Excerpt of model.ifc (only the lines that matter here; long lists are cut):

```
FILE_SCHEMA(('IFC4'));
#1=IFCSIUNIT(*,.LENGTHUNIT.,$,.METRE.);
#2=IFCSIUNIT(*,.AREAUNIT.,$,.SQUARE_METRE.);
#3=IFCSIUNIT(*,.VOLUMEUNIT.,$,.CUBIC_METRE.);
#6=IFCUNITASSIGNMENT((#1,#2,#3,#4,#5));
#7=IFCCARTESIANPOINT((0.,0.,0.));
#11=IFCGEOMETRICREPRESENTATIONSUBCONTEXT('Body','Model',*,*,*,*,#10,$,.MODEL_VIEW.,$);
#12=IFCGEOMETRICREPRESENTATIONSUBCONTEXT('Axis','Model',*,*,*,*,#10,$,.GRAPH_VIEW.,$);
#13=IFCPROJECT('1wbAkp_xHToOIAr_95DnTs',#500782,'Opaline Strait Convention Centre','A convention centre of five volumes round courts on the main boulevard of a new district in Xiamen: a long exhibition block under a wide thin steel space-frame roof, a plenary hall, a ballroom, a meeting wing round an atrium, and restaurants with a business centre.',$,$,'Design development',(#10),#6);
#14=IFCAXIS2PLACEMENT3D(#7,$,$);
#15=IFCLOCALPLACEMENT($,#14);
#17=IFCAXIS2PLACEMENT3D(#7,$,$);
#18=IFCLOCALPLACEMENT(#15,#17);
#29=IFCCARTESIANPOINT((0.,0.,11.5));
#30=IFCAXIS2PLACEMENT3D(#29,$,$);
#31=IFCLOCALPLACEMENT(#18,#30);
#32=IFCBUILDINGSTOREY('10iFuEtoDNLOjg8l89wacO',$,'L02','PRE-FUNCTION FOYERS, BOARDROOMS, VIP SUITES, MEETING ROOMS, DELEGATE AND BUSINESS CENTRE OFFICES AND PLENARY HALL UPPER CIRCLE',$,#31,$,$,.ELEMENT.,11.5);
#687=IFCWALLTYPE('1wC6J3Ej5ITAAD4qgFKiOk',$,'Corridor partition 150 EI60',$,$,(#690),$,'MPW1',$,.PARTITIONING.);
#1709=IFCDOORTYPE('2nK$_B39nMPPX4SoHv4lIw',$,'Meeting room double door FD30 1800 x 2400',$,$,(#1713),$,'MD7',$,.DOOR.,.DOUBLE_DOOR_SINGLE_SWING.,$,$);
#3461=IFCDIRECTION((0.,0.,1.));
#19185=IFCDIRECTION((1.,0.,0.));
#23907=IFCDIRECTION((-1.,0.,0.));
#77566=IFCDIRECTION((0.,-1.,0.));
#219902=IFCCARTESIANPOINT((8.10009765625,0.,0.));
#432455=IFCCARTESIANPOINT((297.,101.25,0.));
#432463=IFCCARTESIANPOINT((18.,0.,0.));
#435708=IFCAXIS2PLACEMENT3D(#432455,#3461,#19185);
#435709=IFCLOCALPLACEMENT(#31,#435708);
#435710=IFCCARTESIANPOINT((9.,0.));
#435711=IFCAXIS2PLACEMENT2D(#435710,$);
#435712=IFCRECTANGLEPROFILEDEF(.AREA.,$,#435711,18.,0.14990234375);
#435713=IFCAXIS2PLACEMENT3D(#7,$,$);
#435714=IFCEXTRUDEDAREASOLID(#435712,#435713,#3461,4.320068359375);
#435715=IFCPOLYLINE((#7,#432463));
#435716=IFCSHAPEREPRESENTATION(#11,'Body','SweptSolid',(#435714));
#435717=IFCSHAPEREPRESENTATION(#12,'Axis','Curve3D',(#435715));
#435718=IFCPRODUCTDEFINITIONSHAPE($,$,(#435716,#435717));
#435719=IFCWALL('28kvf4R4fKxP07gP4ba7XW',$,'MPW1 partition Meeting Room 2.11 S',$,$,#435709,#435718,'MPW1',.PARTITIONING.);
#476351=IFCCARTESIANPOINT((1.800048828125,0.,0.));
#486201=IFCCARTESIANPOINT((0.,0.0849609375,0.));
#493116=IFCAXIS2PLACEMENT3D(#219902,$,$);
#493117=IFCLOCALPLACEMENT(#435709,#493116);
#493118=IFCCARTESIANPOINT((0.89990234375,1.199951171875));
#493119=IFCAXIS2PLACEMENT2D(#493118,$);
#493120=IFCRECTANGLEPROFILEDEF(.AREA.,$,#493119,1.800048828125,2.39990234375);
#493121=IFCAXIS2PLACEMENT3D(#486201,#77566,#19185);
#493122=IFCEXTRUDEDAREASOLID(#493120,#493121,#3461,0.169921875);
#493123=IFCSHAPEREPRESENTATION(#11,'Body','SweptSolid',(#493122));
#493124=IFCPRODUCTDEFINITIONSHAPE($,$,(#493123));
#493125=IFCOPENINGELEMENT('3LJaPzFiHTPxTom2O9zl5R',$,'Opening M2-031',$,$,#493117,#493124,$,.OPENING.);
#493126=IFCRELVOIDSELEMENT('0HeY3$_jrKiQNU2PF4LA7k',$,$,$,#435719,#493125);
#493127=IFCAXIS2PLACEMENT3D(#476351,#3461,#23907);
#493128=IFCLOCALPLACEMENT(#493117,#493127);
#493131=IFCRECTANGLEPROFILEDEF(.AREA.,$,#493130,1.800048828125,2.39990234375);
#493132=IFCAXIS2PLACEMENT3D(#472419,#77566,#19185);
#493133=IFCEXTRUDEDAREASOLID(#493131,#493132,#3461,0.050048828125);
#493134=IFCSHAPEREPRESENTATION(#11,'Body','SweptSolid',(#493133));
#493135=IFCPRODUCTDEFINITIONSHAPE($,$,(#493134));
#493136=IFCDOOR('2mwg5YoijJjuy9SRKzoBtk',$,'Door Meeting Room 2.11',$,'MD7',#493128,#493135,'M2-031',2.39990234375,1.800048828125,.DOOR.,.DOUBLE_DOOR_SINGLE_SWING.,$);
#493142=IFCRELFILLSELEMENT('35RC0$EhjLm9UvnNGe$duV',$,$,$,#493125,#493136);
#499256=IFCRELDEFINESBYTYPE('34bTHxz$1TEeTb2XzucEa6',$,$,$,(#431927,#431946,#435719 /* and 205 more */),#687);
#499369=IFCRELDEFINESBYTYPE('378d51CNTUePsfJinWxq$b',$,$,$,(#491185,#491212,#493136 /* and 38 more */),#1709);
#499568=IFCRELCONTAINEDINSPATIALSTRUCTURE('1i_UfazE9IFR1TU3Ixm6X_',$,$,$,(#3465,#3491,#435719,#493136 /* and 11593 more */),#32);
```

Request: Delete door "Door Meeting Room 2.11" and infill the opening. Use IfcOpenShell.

```python
import ifcopenshell
import ifcopenshell.api.feature
import ifcopenshell.api.root
import ifcopenshell.geom
import ifcopenshell.util.shape

model = ifcopenshell.open("model.ifc")
settings = ifcopenshell.geom.settings()


def volume(element):
    """Net volume in cubic metres, openings subtracted."""
    shape = ifcopenshell.geom.create_shape(settings, element)
    return ifcopenshell.util.shape.get_volume(shape.geometry)


door = model.by_guid("2mwg5YoijJjuy9SRKzoBtk")
opening = door.FillsVoids[0].RelatingOpeningElement
wall = opening.VoidsElements[0].RelatingBuildingElement
before = volume(wall)

ifcopenshell.api.root.remove_product(model, product=door)
ifcopenshell.api.feature.remove_feature(model, feature=opening)

after = volume(wall)

print(f"wall volume {before:.3f} -> {after:.3f} m3")

model.write("model_edited.ifc")
```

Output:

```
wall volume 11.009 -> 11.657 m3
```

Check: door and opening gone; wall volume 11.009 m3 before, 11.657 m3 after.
